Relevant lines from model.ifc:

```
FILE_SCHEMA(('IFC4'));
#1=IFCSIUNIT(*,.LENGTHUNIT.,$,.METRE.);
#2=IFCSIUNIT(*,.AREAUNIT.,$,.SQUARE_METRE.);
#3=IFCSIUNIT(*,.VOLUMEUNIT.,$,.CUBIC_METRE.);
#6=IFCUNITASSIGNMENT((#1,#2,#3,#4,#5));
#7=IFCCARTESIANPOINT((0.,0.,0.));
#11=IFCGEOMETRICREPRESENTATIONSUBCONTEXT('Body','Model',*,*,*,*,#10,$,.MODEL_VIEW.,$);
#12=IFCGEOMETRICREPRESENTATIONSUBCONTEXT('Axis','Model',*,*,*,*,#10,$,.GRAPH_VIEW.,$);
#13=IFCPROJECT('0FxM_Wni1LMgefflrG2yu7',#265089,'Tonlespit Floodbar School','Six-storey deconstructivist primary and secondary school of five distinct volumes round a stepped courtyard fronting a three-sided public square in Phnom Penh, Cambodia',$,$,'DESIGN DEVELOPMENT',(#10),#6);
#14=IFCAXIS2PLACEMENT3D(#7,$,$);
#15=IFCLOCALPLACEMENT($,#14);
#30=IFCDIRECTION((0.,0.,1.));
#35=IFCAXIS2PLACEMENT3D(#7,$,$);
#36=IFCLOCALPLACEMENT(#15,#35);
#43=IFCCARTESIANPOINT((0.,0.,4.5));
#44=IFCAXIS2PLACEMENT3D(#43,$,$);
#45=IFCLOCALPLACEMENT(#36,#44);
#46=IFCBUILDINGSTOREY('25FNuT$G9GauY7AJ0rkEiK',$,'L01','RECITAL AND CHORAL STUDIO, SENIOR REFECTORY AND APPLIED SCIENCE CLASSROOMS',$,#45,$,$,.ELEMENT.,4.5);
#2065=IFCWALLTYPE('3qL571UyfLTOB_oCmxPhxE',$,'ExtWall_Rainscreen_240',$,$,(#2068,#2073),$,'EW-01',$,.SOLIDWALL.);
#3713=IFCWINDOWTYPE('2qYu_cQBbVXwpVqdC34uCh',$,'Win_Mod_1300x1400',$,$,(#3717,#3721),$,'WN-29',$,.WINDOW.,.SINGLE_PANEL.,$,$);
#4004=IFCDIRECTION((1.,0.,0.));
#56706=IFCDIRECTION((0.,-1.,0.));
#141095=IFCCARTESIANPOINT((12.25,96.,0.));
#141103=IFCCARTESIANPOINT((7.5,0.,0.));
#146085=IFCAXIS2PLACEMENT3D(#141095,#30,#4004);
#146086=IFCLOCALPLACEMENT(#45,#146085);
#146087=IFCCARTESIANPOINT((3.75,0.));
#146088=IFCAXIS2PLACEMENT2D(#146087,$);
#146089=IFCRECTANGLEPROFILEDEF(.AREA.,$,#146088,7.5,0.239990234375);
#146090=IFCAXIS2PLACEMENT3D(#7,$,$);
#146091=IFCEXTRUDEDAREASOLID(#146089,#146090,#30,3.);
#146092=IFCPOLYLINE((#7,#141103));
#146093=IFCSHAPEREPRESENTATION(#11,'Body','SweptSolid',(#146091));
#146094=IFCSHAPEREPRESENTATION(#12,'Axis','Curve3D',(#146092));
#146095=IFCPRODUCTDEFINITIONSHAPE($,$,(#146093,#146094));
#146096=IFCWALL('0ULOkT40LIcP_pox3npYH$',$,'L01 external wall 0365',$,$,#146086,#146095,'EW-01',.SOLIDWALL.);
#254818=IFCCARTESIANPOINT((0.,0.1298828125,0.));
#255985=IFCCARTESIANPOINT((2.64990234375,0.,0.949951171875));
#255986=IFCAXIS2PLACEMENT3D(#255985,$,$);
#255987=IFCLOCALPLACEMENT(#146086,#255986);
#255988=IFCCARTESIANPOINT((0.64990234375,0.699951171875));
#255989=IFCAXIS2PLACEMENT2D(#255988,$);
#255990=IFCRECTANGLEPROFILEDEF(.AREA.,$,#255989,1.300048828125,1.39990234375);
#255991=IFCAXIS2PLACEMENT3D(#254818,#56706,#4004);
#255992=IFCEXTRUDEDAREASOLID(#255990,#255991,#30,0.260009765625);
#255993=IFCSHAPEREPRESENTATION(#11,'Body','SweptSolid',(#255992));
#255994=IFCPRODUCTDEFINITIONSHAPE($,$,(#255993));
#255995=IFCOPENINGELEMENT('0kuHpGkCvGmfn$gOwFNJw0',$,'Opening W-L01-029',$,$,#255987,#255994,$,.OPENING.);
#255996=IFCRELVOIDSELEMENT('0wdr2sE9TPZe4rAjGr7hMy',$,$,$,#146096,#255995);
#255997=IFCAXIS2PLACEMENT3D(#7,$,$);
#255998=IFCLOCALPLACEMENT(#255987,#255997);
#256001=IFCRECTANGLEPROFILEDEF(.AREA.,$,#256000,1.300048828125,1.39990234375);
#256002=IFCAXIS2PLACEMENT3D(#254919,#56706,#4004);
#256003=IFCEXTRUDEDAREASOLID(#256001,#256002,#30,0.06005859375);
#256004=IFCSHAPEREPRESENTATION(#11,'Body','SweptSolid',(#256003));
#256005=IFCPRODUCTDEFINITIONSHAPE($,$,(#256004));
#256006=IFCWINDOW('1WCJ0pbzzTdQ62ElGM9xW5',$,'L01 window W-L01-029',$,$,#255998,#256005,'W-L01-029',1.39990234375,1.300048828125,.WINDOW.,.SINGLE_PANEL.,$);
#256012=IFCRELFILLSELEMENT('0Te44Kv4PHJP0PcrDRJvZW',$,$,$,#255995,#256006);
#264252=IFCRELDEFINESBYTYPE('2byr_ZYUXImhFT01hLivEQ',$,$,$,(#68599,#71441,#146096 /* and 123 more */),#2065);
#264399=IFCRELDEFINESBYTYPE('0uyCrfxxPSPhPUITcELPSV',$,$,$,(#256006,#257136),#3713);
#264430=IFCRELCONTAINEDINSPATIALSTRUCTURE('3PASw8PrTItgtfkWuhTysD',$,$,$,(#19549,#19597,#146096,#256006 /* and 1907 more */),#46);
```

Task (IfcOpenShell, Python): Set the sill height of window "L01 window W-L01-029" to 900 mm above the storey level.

```python
import numpy as np
import ifcopenshell
import ifcopenshell.api.geometry
import ifcopenshell.geom
import ifcopenshell.util.element
import ifcopenshell.util.placement
import ifcopenshell.util.shape
import ifcopenshell.util.unit

model = ifcopenshell.open("model.ifc")
unit_scale = ifcopenshell.util.unit.calculate_unit_scale(model)

window = model.by_id(256006)
opening = window.FillsVoids[0].RelatingOpeningElement
storey = ifcopenshell.util.element.get_container(window, ifc_class="IfcBuildingStorey")
level = ifcopenshell.util.placement.get_local_placement(storey.ObjectPlacement)[2, 3]

# The opening's origin need not be at the sill, so measure its lowest point.
shape = ifcopenshell.geom.create_shape(ifcopenshell.geom.settings(), opening)
bottom = ifcopenshell.util.shape.get_shape_bottom_elevation(shape, shape.geometry) / unit_scale
dz = level + 0.9 - bottom

shift = np.array([0.0, 0.0, dz])
# The window is placed relative to its opening, so it follows when the opening moves.
matrix = ifcopenshell.util.placement.get_local_placement(opening.ObjectPlacement)
matrix[:3, 3] += shift
ifcopenshell.api.geometry.edit_object_placement(
    model, product=opening, matrix=matrix, is_si=False, should_transform_children=True
)

print(f"moved by {dz * unit_scale:+.3f} m")

model.write("model_updated.ifc")
```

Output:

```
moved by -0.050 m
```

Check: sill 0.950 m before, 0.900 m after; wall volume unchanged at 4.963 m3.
